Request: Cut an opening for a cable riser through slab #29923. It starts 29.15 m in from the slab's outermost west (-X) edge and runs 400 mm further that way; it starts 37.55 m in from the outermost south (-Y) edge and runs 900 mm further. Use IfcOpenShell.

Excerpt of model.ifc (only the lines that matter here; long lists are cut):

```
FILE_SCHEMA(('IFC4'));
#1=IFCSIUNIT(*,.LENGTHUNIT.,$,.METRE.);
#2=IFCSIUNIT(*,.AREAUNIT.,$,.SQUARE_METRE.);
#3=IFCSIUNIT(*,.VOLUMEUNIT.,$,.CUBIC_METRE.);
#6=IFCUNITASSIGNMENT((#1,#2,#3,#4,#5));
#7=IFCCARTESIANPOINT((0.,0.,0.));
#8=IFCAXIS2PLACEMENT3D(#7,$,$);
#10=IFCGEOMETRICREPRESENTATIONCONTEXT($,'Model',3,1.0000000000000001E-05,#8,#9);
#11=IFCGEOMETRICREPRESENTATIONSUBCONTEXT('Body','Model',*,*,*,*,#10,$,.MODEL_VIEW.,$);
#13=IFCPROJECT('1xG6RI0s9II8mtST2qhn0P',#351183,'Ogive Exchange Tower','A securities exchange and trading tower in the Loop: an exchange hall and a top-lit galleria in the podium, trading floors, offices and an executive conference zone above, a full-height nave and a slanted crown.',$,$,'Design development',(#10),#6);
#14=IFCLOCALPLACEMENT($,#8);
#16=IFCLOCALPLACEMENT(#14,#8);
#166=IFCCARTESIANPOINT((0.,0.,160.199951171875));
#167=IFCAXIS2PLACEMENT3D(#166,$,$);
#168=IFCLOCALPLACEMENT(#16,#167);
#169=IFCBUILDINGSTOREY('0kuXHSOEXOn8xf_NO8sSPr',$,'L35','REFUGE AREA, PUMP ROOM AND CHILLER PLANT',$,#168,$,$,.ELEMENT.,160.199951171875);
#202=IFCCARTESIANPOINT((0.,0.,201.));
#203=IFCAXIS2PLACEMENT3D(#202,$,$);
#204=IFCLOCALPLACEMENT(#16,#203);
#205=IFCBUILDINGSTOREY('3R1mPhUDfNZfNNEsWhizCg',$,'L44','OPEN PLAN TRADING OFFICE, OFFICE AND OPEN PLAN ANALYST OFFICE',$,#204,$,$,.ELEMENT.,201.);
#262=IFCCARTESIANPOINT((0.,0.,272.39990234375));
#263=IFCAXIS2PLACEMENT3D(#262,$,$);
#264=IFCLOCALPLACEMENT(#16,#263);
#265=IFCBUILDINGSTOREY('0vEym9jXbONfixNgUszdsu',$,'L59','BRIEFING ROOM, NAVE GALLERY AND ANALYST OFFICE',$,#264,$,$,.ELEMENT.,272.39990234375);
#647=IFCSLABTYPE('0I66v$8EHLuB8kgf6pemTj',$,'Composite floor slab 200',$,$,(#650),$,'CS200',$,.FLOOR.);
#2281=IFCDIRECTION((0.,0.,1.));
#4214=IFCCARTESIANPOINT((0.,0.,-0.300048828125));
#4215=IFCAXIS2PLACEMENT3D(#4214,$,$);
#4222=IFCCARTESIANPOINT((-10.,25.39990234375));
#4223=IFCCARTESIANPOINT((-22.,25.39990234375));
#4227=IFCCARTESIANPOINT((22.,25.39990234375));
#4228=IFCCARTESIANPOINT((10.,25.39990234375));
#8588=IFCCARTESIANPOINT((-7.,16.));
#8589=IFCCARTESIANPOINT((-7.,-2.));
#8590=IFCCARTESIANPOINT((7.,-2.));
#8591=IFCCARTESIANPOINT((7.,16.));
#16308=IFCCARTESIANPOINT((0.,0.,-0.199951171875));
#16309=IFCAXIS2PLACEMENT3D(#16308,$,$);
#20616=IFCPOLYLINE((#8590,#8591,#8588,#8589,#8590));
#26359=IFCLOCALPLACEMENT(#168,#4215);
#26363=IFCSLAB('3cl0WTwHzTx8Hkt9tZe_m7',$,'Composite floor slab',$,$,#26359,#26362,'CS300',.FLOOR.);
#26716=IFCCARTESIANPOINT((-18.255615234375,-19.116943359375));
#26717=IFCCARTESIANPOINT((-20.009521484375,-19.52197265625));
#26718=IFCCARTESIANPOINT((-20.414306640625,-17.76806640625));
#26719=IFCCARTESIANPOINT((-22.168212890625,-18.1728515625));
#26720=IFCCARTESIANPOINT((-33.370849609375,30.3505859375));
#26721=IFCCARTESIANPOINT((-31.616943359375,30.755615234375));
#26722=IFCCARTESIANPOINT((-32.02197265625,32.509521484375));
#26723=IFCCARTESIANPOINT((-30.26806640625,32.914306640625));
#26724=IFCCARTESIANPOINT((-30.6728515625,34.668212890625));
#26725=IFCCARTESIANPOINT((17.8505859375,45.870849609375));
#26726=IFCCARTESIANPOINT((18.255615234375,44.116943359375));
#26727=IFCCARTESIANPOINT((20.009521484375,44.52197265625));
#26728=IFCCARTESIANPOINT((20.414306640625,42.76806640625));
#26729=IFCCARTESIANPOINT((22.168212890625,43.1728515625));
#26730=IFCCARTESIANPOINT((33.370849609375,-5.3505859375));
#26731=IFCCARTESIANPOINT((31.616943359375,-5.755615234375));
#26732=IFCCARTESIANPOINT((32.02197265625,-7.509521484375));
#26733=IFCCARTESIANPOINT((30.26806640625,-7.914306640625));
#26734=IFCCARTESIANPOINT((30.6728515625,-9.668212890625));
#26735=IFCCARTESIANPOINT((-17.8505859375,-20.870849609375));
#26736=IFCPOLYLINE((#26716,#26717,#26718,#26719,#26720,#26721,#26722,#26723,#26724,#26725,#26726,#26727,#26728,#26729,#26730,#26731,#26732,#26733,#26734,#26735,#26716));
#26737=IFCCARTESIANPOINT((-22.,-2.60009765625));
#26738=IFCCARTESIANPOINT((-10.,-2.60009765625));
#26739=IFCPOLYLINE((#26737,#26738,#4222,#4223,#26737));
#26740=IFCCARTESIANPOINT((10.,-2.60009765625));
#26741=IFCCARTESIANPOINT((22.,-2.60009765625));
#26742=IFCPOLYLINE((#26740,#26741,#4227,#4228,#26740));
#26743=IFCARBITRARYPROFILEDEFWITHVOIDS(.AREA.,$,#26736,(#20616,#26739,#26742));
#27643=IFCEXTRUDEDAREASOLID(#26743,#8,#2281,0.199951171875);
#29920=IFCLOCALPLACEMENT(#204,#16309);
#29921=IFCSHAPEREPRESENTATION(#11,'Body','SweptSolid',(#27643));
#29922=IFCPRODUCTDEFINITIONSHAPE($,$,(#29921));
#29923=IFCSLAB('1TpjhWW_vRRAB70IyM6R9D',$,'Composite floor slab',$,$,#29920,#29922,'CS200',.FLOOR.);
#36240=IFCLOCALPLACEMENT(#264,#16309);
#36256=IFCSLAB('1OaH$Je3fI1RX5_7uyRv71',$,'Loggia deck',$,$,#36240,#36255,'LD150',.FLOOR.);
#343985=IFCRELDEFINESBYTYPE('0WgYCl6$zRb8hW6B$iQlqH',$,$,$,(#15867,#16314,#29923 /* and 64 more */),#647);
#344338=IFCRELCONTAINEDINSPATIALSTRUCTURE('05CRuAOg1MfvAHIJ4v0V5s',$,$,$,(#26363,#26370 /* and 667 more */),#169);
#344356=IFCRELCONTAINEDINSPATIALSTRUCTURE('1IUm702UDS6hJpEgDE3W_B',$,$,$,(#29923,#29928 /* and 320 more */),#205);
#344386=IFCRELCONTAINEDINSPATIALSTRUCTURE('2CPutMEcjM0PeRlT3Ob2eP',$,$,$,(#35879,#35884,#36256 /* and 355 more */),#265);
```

```python
import numpy as np
import ifcopenshell
import ifcopenshell.api.feature
import ifcopenshell.api.geometry
import ifcopenshell.api.root
import ifcopenshell.geom
import ifcopenshell.util.placement
import ifcopenshell.util.representation
import ifcopenshell.util.shape
import ifcopenshell.util.unit

model = ifcopenshell.open("model.ifc")
unit_scale = ifcopenshell.util.unit.calculate_unit_scale(model)
settings = ifcopenshell.geom.settings()


def volume(element):
    """Net volume in cubic metres, openings subtracted."""
    shape = ifcopenshell.geom.create_shape(settings, element)
    return ifcopenshell.util.shape.get_volume(shape.geometry)


slab = model.by_guid("1TpjhWW_vRRAB70IyM6R9D")
before = volume(slab)

# Extent in the slab's own axes, in metres. The edges named are its -X and -Y sides.
slab_shape = ifcopenshell.geom.create_shape(settings, slab)
vertices = ifcopenshell.util.shape.get_vertices(slab_shape.geometry)
x_min, y_min, bottom = vertices.min(axis=0)
top = vertices[:, 2].max()

opening = ifcopenshell.api.root.create_entity(model, ifc_class="IfcOpeningElement", name="Cable riser opening", predefined_type="OPENING")
context = ifcopenshell.util.representation.get_context(model, "Model", "Body", "MODEL_VIEW")
width, depth = 0.4, 0.9
outline = [(0.0, 0.0), (width, 0.0), (width, depth), (0.0, depth), (0.0, 0.0)]
# Overshoot both faces by 50 mm so the cut is clean.
shape = ifcopenshell.api.geometry.add_slab_representation(
    model, context=context, depth=top - bottom + 0.1, polyline=outline
)
ifcopenshell.api.geometry.assign_representation(model, product=opening, representation=shape)

matrix = ifcopenshell.util.placement.get_local_placement(slab.ObjectPlacement)
matrix[:, 3] = matrix @ np.append(np.array([x_min + 29.15, y_min + 37.55, bottom - 0.05]) / unit_scale, 1.0)
ifcopenshell.api.geometry.edit_object_placement(model, product=opening, matrix=matrix, is_si=False)
ifcopenshell.api.feature.add_feature(model, feature=opening, element=slab)

after = volume(slab)

print(f"slab volume {before:.3f} -> {after:.3f} m3")

model.write("model_edited.ifc")
```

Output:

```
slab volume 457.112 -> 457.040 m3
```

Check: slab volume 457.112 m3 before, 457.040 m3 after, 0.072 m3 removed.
